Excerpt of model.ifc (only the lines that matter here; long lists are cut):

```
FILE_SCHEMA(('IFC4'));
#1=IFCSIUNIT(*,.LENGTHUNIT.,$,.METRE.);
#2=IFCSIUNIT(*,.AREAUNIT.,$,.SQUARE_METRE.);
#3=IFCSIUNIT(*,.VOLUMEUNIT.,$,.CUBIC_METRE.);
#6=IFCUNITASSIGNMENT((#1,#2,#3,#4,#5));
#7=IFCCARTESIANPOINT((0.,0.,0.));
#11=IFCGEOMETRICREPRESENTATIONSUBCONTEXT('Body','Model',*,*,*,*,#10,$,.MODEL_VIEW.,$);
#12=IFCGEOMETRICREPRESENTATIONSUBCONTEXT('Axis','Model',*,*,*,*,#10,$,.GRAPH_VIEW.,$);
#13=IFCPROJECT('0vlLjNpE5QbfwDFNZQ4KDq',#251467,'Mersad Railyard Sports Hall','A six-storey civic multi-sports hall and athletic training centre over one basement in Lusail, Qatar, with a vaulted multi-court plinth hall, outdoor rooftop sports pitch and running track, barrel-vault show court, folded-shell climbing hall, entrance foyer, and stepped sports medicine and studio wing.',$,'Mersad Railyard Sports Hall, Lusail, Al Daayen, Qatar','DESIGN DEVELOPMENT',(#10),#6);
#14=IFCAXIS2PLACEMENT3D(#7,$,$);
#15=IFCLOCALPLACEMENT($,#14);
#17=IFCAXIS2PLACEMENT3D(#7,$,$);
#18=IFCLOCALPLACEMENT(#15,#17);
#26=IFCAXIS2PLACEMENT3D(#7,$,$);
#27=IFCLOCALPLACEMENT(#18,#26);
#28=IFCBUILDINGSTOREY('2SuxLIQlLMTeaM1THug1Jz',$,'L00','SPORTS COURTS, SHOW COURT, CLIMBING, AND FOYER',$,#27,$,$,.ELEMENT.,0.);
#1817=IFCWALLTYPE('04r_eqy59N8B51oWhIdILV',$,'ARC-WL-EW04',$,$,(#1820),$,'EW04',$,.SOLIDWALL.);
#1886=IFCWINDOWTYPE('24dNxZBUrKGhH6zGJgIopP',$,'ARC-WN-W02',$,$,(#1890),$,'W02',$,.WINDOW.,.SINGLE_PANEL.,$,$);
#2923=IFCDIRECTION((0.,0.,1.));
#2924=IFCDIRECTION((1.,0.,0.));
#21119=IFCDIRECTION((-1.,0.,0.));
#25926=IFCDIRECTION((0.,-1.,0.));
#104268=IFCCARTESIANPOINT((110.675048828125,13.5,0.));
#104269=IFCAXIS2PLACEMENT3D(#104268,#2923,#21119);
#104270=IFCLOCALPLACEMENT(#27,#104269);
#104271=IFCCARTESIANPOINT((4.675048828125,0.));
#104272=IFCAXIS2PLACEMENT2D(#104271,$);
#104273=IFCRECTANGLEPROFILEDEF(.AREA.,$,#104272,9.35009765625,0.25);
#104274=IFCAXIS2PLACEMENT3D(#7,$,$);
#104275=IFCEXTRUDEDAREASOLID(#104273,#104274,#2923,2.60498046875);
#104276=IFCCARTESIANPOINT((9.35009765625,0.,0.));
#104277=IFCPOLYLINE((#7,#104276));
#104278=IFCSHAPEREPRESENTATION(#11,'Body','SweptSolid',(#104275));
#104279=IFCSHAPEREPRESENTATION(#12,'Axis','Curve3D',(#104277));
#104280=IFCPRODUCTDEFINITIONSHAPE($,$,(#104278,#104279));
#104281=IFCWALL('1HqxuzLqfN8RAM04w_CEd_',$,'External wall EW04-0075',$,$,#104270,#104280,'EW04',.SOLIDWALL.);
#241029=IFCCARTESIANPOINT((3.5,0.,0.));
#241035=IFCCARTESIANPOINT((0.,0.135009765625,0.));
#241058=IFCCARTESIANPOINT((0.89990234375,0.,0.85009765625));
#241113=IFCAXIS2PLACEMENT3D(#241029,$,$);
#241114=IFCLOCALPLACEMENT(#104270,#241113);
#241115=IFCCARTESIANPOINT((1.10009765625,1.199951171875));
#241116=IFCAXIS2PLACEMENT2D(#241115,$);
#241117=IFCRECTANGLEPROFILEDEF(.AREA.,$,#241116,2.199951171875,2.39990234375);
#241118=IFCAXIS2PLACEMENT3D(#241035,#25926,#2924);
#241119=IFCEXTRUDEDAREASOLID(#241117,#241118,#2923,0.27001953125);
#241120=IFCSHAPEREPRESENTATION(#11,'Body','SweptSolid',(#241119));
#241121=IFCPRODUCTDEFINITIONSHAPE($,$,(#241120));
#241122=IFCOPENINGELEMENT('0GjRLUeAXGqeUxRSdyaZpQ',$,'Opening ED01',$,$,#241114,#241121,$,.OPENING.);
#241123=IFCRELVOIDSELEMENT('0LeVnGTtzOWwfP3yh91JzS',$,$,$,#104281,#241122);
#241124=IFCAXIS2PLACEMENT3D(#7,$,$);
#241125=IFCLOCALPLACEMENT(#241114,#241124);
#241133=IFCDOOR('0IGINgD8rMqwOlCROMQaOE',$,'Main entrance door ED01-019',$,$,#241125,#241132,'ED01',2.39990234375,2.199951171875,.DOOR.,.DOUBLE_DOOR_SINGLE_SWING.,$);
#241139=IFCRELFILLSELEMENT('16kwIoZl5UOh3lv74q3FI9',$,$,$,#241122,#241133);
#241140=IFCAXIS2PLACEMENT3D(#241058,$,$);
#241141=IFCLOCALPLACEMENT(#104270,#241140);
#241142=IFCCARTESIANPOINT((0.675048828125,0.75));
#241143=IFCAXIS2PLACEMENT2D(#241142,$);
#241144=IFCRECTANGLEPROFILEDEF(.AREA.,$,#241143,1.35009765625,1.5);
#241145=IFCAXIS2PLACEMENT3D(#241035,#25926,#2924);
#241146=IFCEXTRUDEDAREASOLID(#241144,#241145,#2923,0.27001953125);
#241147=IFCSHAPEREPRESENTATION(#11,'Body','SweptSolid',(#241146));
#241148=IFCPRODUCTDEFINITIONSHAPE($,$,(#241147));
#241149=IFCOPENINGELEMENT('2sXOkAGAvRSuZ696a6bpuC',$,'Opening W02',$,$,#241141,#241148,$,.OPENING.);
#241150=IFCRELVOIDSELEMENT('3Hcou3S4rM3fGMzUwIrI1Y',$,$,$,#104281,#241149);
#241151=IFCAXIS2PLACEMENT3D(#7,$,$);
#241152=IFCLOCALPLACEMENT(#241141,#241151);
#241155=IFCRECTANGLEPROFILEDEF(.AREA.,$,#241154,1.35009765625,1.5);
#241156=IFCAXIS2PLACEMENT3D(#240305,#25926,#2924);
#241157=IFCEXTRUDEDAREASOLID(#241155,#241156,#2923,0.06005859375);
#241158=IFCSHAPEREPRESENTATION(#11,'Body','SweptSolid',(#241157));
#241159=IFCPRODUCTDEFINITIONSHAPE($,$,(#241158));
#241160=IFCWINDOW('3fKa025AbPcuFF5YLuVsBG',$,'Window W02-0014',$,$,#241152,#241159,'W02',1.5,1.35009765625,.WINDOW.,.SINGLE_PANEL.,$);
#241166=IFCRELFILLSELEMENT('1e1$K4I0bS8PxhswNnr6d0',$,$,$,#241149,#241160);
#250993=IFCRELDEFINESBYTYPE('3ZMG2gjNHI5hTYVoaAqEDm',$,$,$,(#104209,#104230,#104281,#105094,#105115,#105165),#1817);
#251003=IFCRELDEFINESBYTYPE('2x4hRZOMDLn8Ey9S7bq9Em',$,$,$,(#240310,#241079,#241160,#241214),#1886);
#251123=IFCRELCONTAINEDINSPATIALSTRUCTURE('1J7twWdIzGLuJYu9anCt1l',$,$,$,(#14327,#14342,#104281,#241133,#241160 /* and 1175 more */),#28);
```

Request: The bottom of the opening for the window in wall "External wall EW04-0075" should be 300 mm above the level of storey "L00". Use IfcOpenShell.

```python
import numpy as np
import ifcopenshell
import ifcopenshell.api.geometry
import ifcopenshell.geom
import ifcopenshell.util.element
import ifcopenshell.util.placement
import ifcopenshell.util.shape
import ifcopenshell.util.unit

model = ifcopenshell.open("model.ifc")
unit_scale = ifcopenshell.util.unit.calculate_unit_scale(model)

window = model.by_id(241160)
opening = window.FillsVoids[0].RelatingOpeningElement
storey = ifcopenshell.util.element.get_container(window, ifc_class="IfcBuildingStorey")
level = ifcopenshell.util.placement.get_local_placement(storey.ObjectPlacement)[2, 3]

# The opening's origin need not be at the sill, so measure its lowest point.
shape = ifcopenshell.geom.create_shape(ifcopenshell.geom.settings(), opening)
bottom = ifcopenshell.util.shape.get_shape_bottom_elevation(shape, shape.geometry) / unit_scale
dz = level + 0.3 / unit_scale - bottom

shift = np.array([0.0, 0.0, dz])
# The window is placed relative to its opening, so it follows when the opening moves.
matrix = ifcopenshell.util.placement.get_local_placement(opening.ObjectPlacement)
matrix[:3, 3] += shift
ifcopenshell.api.geometry.edit_object_placement(
    model, product=opening, matrix=matrix, is_si=False, should_transform_children=True
)

print(f"moved by {dz * unit_scale:+.3f} m")

model.write("model-out.ifc")
```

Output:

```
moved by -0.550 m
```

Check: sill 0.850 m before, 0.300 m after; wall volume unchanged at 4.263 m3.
